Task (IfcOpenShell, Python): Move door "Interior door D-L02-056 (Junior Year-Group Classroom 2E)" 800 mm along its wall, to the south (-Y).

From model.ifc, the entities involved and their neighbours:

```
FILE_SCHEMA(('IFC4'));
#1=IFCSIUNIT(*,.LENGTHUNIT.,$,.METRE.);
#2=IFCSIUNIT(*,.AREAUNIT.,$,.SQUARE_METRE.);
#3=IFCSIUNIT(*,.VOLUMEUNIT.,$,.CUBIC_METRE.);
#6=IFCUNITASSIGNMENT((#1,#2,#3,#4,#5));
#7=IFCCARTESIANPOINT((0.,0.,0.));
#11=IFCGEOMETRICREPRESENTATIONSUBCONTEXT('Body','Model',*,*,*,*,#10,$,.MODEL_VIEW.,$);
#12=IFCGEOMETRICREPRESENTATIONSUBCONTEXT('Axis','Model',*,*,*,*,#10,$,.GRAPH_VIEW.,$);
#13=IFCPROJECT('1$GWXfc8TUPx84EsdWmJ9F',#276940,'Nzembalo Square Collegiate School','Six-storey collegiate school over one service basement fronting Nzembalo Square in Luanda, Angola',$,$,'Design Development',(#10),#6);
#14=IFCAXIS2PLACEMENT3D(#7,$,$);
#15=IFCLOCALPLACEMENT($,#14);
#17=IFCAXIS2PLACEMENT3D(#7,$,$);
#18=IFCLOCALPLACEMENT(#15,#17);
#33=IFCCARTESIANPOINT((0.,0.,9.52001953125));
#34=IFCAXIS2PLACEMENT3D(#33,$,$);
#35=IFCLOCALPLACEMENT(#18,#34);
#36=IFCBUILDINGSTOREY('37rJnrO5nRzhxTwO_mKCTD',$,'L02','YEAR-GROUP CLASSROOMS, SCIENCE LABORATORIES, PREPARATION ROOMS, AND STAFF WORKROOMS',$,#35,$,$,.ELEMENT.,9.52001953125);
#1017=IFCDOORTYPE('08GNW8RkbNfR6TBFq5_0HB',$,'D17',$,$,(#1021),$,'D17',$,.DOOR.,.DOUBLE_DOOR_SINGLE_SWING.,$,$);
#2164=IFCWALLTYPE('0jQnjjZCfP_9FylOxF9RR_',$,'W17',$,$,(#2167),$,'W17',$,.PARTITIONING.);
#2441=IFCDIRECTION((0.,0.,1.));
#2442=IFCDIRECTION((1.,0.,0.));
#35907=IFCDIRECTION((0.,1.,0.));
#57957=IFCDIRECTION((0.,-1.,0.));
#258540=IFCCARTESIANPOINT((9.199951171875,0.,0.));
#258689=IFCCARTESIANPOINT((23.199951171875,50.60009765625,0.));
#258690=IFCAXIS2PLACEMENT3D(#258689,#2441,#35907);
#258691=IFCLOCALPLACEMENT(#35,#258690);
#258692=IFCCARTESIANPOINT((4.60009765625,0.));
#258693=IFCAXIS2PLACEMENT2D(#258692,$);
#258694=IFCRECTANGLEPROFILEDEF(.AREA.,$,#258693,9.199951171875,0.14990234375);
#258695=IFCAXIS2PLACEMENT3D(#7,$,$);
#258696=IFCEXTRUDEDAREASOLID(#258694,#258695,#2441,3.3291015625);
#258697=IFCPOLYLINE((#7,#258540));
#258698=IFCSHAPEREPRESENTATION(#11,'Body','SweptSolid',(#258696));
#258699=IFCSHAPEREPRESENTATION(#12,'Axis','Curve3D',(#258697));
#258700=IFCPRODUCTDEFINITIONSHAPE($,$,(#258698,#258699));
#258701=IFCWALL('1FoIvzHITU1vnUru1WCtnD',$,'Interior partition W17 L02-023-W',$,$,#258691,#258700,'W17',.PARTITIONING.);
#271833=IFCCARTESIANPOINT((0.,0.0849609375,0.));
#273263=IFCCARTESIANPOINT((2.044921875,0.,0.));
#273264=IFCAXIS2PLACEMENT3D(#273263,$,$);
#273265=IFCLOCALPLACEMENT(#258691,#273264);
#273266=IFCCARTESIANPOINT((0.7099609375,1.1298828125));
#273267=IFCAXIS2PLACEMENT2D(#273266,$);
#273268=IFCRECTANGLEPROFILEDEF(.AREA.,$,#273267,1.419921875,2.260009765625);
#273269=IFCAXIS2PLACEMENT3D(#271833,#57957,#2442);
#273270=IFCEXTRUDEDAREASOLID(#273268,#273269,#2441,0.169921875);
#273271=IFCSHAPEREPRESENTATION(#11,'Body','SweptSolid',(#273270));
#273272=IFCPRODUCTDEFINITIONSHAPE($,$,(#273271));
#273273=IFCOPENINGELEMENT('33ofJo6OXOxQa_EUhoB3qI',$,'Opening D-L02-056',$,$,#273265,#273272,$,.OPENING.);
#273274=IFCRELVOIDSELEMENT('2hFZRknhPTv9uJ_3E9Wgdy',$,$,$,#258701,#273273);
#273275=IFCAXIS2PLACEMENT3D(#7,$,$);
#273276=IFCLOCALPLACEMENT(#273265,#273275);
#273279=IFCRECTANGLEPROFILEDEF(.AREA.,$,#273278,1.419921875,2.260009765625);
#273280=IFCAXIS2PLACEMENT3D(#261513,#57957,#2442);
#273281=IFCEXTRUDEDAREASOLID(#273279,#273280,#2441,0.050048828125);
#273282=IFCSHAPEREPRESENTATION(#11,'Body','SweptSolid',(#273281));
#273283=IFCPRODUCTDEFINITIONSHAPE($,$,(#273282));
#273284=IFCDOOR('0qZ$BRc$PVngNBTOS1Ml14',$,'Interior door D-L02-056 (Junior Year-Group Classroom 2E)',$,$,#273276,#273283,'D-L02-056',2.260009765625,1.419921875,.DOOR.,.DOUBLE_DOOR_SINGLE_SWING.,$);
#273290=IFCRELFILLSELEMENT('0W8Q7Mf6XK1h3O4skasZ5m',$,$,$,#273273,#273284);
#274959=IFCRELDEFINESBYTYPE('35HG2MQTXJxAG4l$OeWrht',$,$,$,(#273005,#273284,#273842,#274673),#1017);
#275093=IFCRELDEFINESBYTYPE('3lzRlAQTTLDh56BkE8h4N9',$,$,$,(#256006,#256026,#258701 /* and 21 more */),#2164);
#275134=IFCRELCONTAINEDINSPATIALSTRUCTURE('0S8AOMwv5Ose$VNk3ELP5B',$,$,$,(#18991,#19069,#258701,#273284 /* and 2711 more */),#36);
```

```python
import ifcopenshell
import ifcopenshell.api.geometry
import ifcopenshell.util.placement
import ifcopenshell.util.unit

model = ifcopenshell.open("model.ifc")
unit_scale = ifcopenshell.util.unit.calculate_unit_scale(model)

door = model.by_guid("0qZ$BRc$PVngNBTOS1Ml14")
opening = door.FillsVoids[0].RelatingOpeningElement
wall = opening.VoidsElements[0].RelatingBuildingElement

wall_matrix = ifcopenshell.util.placement.get_local_placement(wall.ObjectPlacement)
shift = wall_matrix[:3, 0] * -0.8 / unit_scale
before = ifcopenshell.util.placement.get_local_placement(door.ObjectPlacement)[:3, 3].copy()

# The door is placed relative to its opening, so it follows when the opening moves.
matrix = ifcopenshell.util.placement.get_local_placement(opening.ObjectPlacement)
matrix[:3, 3] += shift
ifcopenshell.api.geometry.edit_object_placement(
    model, product=opening, matrix=matrix, is_si=False, should_transform_children=True
)

after = ifcopenshell.util.placement.get_local_placement(door.ObjectPlacement)[:3, 3]
print("door moved by", (after - before).round(3) + 0.0)

model.write("model_v2.ifc")
```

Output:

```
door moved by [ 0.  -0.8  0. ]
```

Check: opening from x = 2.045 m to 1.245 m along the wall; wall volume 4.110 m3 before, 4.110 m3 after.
